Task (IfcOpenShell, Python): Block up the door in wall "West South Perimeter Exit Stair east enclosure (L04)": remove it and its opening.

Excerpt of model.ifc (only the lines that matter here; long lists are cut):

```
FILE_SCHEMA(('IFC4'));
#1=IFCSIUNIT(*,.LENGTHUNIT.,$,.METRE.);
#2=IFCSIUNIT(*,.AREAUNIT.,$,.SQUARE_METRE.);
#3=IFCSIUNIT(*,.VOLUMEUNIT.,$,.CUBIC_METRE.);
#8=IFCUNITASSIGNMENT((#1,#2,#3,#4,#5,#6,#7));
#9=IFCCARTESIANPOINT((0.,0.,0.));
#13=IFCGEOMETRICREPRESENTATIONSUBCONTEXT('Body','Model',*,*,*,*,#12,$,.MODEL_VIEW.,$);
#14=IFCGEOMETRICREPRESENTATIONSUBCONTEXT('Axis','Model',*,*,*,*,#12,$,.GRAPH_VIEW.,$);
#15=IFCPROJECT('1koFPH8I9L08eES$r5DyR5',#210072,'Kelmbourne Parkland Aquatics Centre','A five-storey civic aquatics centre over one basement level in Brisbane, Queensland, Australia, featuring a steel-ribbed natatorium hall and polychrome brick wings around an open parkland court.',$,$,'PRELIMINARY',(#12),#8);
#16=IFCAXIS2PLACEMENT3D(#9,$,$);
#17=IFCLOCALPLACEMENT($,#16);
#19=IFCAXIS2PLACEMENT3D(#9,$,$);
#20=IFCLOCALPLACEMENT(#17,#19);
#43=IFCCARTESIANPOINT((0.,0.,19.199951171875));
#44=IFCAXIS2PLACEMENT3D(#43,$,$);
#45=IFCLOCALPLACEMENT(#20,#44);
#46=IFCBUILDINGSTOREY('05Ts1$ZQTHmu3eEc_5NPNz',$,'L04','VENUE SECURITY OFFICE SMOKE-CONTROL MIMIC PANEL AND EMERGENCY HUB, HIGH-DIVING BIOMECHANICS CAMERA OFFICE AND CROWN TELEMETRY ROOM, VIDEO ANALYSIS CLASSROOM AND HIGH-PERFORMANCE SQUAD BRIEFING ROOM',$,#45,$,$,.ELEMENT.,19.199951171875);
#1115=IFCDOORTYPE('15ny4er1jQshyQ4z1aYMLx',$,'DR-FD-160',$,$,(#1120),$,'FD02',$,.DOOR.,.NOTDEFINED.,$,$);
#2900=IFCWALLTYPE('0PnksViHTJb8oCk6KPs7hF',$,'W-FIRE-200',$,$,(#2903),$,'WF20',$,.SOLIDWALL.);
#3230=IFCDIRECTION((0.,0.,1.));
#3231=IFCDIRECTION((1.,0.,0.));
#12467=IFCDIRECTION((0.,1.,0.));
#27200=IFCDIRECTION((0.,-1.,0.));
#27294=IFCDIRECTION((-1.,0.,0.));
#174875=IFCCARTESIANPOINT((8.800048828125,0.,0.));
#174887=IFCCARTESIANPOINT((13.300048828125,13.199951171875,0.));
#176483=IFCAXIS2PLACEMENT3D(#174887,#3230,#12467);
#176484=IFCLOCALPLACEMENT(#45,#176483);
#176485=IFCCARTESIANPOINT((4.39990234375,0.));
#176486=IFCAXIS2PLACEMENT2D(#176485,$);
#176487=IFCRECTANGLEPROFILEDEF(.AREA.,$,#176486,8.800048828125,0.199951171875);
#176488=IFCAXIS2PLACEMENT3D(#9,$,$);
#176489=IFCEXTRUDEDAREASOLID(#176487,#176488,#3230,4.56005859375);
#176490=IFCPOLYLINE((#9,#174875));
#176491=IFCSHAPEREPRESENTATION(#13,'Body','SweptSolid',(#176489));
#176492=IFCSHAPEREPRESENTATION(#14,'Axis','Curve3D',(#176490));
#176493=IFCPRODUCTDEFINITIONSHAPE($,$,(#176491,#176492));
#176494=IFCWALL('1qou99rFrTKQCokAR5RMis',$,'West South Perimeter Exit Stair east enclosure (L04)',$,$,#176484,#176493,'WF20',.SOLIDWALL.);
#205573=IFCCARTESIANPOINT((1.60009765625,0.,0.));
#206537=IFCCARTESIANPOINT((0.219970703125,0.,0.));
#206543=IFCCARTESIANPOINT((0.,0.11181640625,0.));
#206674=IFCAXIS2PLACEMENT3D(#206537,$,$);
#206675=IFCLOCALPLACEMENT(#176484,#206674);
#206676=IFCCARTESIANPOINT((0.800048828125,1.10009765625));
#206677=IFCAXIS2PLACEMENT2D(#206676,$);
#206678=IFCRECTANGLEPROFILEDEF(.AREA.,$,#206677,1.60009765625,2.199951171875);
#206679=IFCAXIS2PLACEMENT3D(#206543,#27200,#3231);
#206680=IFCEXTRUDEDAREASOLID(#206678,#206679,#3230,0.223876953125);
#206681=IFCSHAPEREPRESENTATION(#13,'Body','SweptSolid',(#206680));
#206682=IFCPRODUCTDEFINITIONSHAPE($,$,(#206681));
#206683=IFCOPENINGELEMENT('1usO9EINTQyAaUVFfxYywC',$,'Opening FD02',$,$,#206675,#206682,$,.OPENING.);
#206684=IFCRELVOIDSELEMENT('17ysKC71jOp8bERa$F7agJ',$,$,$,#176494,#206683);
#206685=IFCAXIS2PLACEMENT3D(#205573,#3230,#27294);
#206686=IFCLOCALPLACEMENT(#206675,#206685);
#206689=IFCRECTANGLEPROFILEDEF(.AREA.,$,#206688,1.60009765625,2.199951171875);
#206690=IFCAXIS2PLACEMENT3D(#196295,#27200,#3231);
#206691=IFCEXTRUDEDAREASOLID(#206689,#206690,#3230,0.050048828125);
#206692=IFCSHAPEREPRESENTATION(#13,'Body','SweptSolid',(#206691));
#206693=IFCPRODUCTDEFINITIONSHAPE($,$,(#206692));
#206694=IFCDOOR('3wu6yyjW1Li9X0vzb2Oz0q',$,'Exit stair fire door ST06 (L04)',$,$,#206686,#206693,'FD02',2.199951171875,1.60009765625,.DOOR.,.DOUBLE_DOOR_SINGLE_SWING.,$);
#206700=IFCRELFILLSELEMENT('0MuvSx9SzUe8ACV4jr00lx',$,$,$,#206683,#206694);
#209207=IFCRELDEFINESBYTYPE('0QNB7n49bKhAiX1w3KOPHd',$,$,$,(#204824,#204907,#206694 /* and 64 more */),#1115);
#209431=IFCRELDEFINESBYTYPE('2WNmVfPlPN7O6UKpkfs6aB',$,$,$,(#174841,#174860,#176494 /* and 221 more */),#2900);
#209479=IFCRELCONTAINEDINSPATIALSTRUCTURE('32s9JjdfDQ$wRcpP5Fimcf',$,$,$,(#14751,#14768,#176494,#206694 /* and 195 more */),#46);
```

```python
import ifcopenshell
import ifcopenshell.api.feature
import ifcopenshell.api.root
import ifcopenshell.geom
import ifcopenshell.util.shape

model = ifcopenshell.open("model.ifc")
settings = ifcopenshell.geom.settings()


def volume(element):
    """Net volume in cubic metres, openings subtracted."""
    shape = ifcopenshell.geom.create_shape(settings, element)
    return ifcopenshell.util.shape.get_volume(shape.geometry)


door = model.by_id(206694)
opening = door.FillsVoids[0].RelatingOpeningElement
wall = opening.VoidsElements[0].RelatingBuildingElement
before = volume(wall)

ifcopenshell.api.root.remove_product(model, product=door)
ifcopenshell.api.feature.remove_feature(model, feature=opening)

after = volume(wall)

print(f"wall volume {before:.3f} -> {after:.3f} m3")

model.write("model_rev.ifc")
```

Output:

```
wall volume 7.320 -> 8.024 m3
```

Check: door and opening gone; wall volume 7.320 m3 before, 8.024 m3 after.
